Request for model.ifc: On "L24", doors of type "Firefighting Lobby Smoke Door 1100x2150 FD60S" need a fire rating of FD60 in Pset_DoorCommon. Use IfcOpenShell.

First a look at what the model holds.

```python
import ifcopenshell
import ifcopenshell.util.element

model = ifcopenshell.open("model.ifc")
print(model.schema)
storey = next(s for s in model.by_type("IfcBuildingStorey") if s.Name == "L24")
doors = [e for e in ifcopenshell.util.element.get_decomposition(storey) if e.is_a("IfcDoor")]
seen = {}
for e in doors:
    element_type = ifcopenshell.util.element.get_type(e)
    key = (element_type.Name if element_type != e and element_type else None, ifcopenshell.util.element.get_pset(e, "Pset_DoorCommon", "FireRating"))
    seen[key] = seen.get(key, 0) + 1
for (name, value), count in sorted(seen.items(), key=str):
    print(count, "x", name, "|", value)
```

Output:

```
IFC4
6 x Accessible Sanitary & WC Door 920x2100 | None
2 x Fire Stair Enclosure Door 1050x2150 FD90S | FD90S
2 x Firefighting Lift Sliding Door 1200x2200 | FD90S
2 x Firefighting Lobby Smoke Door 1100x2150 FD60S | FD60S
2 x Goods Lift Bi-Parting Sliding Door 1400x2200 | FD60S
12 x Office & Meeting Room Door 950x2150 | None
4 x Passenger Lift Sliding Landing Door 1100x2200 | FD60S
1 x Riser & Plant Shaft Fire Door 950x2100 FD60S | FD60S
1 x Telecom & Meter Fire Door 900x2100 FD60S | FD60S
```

```python
import ifcopenshell
import ifcopenshell.api.pset
import ifcopenshell.util.element

model = ifcopenshell.open("model.ifc")

storey = next(s for s in model.by_type("IfcBuildingStorey") if s.Name == "L24")
doors = [e for e in ifcopenshell.util.element.get_decomposition(storey) if e.is_a("IfcDoor")]

count = 0
for e in doors:
    element_type = ifcopenshell.util.element.get_type(e)
    if element_type in (None, e) or element_type.Name != "Firefighting Lobby Smoke Door 1100x2150 FD60S":
        continue
    # add_pset returns the element's existing set when there is one.
    pset = ifcopenshell.api.pset.add_pset(model, product=e, name="Pset_DoorCommon")
    ifcopenshell.api.pset.edit_pset(model, pset=pset, properties={"FireRating": "FD60"})
    count += 1

print(count, "doors updated")

model.write("model_updated.ifc")
```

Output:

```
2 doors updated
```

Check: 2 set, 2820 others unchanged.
